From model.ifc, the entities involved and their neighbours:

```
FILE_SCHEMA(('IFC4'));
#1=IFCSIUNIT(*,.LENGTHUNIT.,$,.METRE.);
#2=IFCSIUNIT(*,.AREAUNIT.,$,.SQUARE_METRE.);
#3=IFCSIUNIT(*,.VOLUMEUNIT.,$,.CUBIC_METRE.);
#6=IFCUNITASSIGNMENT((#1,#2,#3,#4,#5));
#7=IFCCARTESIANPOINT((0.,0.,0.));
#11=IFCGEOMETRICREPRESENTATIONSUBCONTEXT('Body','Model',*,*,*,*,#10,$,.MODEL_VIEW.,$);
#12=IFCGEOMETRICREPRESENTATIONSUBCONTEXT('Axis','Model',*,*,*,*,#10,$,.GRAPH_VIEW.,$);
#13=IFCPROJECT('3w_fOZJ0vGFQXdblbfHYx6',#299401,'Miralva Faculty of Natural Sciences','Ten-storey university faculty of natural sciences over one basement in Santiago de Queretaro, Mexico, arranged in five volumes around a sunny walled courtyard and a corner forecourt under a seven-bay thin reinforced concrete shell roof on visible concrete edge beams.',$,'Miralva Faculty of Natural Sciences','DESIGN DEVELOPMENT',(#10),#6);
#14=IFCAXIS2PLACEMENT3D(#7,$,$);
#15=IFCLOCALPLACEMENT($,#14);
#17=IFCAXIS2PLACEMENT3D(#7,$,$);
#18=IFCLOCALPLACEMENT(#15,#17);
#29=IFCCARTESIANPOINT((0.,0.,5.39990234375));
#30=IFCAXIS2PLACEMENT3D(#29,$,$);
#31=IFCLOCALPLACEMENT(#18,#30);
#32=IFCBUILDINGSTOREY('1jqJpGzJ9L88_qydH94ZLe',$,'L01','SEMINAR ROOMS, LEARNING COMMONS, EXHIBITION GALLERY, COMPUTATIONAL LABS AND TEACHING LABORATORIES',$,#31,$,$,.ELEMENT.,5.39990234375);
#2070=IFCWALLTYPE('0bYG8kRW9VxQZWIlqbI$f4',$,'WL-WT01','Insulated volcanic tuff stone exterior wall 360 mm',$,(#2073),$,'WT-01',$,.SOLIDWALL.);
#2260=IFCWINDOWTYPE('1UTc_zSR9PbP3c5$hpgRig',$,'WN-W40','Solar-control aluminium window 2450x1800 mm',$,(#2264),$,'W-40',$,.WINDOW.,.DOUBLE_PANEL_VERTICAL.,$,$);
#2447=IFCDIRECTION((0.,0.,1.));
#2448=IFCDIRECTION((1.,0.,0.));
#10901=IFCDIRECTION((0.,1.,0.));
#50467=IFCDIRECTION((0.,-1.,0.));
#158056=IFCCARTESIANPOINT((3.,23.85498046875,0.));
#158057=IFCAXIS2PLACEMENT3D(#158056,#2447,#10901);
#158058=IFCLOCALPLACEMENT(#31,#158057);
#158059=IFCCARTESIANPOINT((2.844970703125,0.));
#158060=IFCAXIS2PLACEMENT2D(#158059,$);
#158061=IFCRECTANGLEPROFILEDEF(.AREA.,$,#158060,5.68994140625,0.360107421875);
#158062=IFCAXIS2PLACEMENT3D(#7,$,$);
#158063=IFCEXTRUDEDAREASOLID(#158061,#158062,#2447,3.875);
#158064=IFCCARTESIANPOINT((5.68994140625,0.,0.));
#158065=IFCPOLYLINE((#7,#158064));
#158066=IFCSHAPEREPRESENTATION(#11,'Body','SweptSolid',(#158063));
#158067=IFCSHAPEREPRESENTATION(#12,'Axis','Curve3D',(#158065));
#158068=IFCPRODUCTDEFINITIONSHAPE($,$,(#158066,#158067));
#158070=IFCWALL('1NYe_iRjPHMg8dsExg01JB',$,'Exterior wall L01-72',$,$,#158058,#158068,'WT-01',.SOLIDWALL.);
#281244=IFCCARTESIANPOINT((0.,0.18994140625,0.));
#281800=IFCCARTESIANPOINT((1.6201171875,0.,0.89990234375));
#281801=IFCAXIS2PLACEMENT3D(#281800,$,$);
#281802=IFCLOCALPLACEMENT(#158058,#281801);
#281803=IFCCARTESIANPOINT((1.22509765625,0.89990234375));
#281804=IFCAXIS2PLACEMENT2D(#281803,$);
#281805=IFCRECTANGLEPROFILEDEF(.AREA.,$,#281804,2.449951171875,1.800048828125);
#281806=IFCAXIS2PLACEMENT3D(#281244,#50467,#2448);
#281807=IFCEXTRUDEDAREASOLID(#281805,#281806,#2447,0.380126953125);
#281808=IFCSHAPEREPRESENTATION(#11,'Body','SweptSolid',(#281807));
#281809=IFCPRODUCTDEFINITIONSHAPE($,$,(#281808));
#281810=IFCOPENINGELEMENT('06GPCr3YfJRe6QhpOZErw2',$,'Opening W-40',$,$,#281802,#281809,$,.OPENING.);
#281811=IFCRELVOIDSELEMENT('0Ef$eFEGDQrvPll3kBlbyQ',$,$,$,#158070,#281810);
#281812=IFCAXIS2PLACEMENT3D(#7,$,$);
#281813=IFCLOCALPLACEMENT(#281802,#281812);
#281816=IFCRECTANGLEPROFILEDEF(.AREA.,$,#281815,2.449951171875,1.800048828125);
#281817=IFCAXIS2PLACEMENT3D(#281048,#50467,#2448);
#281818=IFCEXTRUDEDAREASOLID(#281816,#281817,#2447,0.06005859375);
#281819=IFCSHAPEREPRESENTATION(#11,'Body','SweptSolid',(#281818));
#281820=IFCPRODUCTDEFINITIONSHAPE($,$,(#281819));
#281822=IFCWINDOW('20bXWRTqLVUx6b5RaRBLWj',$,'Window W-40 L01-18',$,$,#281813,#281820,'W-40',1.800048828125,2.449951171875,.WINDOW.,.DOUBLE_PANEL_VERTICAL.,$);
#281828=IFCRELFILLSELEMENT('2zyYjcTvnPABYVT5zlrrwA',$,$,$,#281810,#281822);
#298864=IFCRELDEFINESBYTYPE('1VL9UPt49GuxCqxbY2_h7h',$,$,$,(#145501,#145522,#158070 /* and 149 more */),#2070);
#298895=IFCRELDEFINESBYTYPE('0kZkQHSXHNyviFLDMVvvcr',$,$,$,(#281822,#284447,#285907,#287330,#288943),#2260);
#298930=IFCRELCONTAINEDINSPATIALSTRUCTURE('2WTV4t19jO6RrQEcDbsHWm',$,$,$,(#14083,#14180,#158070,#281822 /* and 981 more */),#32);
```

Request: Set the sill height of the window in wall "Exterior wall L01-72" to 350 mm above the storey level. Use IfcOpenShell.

```python
import numpy as np
import ifcopenshell
import ifcopenshell.api.geometry
import ifcopenshell.geom
import ifcopenshell.util.element
import ifcopenshell.util.placement
import ifcopenshell.util.shape
import ifcopenshell.util.unit

model = ifcopenshell.open("model.ifc")
unit_scale = ifcopenshell.util.unit.calculate_unit_scale(model)

window = model.by_guid("20bXWRTqLVUx6b5RaRBLWj")
opening = window.FillsVoids[0].RelatingOpeningElement
storey = ifcopenshell.util.element.get_container(window, ifc_class="IfcBuildingStorey")
level = ifcopenshell.util.placement.get_local_placement(storey.ObjectPlacement)[2, 3]

# The opening's origin need not be at the sill, so measure its lowest point.
shape = ifcopenshell.geom.create_shape(ifcopenshell.geom.settings(), opening)
bottom = ifcopenshell.util.shape.get_shape_bottom_elevation(shape, shape.geometry) / unit_scale
dz = level + 0.35 / unit_scale - bottom

shift = np.array([0.0, 0.0, dz])
# The window is placed relative to its opening, so it follows when the opening moves.
matrix = ifcopenshell.util.placement.get_local_placement(opening.ObjectPlacement)
matrix[:3, 3] += shift
ifcopenshell.api.geometry.edit_object_placement(
    model, product=opening, matrix=matrix, is_si=False, should_transform_children=True
)

print(f"moved by {dz * unit_scale:+.3f} m")

model.write("model_v2.ifc")
```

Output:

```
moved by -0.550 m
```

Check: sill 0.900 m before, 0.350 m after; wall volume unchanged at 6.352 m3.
